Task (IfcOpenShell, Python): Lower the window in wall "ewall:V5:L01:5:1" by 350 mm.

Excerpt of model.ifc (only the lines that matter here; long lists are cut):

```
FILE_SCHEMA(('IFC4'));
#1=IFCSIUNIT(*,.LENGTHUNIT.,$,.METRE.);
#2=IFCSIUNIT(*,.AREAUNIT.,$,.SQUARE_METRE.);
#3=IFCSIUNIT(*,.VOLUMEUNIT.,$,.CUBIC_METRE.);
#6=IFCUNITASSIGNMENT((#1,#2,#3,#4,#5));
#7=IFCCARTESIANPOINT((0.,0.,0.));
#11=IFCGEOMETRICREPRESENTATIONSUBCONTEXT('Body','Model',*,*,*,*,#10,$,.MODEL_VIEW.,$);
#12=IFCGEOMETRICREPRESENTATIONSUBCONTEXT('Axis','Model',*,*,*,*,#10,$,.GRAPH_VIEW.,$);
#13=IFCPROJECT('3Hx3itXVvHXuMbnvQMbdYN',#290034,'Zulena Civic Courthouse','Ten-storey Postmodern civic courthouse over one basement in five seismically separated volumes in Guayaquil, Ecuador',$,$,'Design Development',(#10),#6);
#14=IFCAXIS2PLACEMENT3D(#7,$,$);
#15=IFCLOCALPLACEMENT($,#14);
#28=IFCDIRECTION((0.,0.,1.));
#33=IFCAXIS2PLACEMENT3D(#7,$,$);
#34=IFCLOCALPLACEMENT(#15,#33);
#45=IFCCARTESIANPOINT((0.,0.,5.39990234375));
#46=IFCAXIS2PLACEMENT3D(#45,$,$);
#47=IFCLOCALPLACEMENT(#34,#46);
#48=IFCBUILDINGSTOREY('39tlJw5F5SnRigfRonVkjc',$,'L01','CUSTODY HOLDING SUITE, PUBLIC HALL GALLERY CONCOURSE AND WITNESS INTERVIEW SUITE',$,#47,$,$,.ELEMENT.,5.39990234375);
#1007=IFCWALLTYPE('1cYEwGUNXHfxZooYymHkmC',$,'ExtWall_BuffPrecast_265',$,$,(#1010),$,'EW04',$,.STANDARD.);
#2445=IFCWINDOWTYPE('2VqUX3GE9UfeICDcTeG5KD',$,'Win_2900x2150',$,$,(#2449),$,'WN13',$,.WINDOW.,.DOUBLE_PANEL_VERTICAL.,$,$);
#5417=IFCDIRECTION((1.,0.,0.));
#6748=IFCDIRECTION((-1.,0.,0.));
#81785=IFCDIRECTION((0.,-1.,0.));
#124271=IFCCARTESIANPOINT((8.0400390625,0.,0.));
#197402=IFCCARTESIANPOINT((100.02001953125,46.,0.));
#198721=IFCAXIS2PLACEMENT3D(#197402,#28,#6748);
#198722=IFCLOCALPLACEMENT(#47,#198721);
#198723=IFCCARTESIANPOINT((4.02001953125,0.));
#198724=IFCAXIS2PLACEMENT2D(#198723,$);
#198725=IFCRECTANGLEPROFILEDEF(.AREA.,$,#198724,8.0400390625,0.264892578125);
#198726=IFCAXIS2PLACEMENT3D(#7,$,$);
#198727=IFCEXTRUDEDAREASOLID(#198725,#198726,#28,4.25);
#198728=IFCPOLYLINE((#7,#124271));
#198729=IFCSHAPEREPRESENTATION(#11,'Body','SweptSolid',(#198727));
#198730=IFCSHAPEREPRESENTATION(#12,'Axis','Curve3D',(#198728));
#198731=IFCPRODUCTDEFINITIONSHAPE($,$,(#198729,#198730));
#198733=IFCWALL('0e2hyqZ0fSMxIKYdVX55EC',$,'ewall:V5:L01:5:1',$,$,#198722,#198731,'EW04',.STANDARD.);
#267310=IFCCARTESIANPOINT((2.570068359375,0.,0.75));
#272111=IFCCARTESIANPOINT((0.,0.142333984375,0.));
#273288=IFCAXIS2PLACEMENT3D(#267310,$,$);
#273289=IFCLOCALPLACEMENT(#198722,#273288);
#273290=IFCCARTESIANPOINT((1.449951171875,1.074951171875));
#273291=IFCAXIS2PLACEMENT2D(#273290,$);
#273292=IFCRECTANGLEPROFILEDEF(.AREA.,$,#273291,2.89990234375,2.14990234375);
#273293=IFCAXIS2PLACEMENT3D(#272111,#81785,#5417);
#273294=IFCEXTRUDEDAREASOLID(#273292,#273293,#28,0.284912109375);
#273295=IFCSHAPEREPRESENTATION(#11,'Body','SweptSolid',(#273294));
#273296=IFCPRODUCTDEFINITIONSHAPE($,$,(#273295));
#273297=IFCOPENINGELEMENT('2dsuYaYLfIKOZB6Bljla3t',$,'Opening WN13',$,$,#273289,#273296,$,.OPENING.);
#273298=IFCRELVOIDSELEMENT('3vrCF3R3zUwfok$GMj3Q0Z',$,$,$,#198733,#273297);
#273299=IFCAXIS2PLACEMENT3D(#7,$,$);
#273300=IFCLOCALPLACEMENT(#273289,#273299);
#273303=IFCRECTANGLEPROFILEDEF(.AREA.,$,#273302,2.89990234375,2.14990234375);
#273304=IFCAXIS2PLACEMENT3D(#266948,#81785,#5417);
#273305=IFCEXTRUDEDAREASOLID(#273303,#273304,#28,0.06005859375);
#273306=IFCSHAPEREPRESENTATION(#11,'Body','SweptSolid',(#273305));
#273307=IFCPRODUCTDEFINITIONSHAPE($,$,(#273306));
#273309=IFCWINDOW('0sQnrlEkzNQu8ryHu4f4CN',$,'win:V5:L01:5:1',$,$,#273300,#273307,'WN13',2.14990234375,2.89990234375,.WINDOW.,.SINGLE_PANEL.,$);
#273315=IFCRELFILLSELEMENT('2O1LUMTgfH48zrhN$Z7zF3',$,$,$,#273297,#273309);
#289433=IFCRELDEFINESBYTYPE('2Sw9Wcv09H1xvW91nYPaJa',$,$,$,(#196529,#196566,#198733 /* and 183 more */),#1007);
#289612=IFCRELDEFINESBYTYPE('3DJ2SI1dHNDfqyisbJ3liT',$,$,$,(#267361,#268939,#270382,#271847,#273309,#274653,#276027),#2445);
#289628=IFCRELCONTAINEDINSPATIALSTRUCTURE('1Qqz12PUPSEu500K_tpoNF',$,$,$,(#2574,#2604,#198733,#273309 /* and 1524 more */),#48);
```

```python
import numpy as np
import ifcopenshell
import ifcopenshell.api.geometry
import ifcopenshell.util.placement
import ifcopenshell.util.unit

model = ifcopenshell.open("model.ifc")
unit_scale = ifcopenshell.util.unit.calculate_unit_scale(model)

window = model.by_guid("0sQnrlEkzNQu8ryHu4f4CN")
opening = window.FillsVoids[0].RelatingOpeningElement
dz = -0.35 / unit_scale

shift = np.array([0.0, 0.0, dz])
# The window is placed relative to its opening, so it follows when the opening moves.
matrix = ifcopenshell.util.placement.get_local_placement(opening.ObjectPlacement)
matrix[:3, 3] += shift
ifcopenshell.api.geometry.edit_object_placement(
    model, product=opening, matrix=matrix, is_si=False, should_transform_children=True
)

print(f"moved by {dz * unit_scale:+.3f} m")

model.write("model_updated.ifc")
```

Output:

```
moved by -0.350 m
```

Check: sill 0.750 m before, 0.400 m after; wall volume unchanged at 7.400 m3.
